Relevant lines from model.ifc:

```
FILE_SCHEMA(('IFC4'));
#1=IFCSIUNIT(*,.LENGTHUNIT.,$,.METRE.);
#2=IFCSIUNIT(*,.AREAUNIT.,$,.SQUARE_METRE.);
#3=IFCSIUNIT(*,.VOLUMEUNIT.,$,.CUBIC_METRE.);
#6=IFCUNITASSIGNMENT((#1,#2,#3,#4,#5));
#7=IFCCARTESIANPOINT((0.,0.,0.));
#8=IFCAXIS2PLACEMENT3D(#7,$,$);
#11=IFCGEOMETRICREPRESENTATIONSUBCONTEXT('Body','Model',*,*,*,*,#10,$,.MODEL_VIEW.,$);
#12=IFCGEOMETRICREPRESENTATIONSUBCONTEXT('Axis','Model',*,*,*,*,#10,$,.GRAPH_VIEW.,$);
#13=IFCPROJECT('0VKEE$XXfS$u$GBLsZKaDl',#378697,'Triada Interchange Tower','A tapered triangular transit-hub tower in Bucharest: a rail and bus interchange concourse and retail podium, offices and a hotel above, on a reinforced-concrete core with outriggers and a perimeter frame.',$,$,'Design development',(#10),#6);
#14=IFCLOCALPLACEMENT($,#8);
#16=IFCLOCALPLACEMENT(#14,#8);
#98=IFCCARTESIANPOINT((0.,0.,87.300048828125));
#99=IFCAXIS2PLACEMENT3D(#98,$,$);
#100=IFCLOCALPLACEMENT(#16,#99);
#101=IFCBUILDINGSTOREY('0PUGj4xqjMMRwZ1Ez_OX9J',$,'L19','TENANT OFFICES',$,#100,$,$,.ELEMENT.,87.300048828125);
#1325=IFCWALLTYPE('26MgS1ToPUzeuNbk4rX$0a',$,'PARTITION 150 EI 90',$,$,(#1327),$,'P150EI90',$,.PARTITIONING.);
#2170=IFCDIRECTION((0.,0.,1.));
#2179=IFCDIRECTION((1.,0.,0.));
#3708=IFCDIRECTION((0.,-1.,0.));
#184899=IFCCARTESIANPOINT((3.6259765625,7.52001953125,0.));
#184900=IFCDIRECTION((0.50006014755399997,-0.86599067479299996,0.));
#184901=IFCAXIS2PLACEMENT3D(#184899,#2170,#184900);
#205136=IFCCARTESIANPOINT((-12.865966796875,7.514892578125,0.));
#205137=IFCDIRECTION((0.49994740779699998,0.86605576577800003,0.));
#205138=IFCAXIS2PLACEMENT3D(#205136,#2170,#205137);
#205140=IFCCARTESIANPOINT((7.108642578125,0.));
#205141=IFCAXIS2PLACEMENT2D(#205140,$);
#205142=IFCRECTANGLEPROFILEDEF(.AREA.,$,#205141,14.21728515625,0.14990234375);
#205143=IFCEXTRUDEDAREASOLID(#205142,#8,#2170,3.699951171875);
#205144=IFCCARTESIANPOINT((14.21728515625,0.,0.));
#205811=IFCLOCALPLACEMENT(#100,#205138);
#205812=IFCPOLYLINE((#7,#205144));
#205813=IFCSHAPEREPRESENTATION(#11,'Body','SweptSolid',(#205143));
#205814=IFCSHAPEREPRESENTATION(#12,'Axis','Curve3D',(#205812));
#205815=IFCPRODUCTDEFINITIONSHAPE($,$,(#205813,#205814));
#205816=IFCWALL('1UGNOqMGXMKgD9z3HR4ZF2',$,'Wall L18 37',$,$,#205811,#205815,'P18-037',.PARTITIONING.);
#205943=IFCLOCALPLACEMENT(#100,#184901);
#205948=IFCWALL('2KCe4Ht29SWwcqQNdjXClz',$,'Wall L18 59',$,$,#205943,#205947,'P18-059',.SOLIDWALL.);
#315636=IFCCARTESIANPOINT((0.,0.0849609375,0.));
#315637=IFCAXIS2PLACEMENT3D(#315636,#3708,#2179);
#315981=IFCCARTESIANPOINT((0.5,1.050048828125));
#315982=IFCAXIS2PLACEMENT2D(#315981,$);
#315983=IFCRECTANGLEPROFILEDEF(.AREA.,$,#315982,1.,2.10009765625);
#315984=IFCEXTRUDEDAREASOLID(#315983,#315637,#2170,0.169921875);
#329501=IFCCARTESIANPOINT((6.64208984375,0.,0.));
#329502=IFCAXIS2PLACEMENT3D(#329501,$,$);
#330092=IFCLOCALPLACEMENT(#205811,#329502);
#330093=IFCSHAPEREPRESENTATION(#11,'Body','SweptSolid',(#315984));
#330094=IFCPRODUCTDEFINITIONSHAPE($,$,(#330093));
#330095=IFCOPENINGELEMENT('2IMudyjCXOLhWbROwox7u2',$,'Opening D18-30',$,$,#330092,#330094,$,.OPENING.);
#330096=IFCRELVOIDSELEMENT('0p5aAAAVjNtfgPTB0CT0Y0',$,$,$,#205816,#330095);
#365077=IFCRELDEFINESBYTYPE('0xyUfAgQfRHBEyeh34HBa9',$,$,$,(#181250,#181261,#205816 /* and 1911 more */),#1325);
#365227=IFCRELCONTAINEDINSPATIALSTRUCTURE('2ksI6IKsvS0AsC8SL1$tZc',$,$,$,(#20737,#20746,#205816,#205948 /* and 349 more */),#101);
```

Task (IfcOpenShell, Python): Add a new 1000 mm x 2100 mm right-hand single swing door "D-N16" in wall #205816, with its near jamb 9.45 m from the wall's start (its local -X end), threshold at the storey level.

```python
import numpy as np
import ifcopenshell
import ifcopenshell.api.feature
import ifcopenshell.api.geometry
import ifcopenshell.api.root
import ifcopenshell.api.spatial
import ifcopenshell.geom
import ifcopenshell.util.element
import ifcopenshell.util.placement
import ifcopenshell.util.representation
import ifcopenshell.util.shape
import ifcopenshell.util.unit

model = ifcopenshell.open("model.ifc")
unit_scale = ifcopenshell.util.unit.calculate_unit_scale(model)
settings = ifcopenshell.geom.settings()


def volume(element):
    """Net volume in cubic metres, openings subtracted."""
    shape = ifcopenshell.geom.create_shape(settings, element)
    return ifcopenshell.util.shape.get_volume(shape.geometry)


wall = model.by_id(205816)
storey = ifcopenshell.util.element.get_container(wall, ifc_class="IfcBuildingStorey")
context = ifcopenshell.util.representation.get_context(model, "Model", "Body", "MODEL_VIEW")
before = volume(wall)

width, height, from_end, sill = 1, 2.1, 9.45, 0.0  # metres

# The wall runs along its own X axis, and the end named is its -X end.
wall_shape = ifcopenshell.geom.create_shape(settings, wall)
x, y, z = ifcopenshell.util.shape.get_vertices(wall_shape.geometry).T
start = x.min() + from_end
face, thickness = float(y.min()), float(y.max() - y.min())
wall_matrix = ifcopenshell.util.placement.get_local_placement(wall.ObjectPlacement)
level = ifcopenshell.util.placement.get_local_placement(storey.ObjectPlacement)[2, 3]


def in_wall(x, y):
    """Placement at x, y metres in the wall's axes, at sill height."""
    matrix = wall_matrix.copy()
    matrix[:, 3] = wall_matrix @ np.array([x / unit_scale, y / unit_scale, 0.0, 1.0])
    matrix[2, 3] = level + sill / unit_scale
    return matrix


# Opening: a box that overshoots both wall faces by 50 mm.
opening = ifcopenshell.api.root.create_entity(model, ifc_class="IfcOpeningElement", predefined_type="OPENING")
box = ifcopenshell.api.geometry.add_wall_representation(
    model, context=context, length=width, height=height, thickness=thickness + 0.1
)
ifcopenshell.api.geometry.assign_representation(model, product=opening, representation=box)
ifcopenshell.api.geometry.edit_object_placement(model, product=opening, matrix=in_wall(start, face - 0.05), is_si=False)
ifcopenshell.api.feature.add_feature(model, feature=opening, element=wall)

door = ifcopenshell.api.root.create_entity(model, ifc_class="IfcDoor", name="D-N16", predefined_type="DOOR")
door.OverallWidth, door.OverallHeight = width / unit_scale, height / unit_scale
door.OperationType = "SINGLE_SWING_RIGHT"
body = ifcopenshell.api.geometry.add_door_representation(
    model,
    context=context,
    overall_width=door.OverallWidth,
    overall_height=door.OverallHeight,
    operation_type="SINGLE_SWING_RIGHT",
    lining_properties={"LiningDepth": thickness / unit_scale, "ThresholdDepth": thickness / unit_scale},
)
ifcopenshell.api.geometry.assign_representation(model, product=door, representation=body)
ifcopenshell.api.spatial.assign_container(model, products=[door], relating_structure=storey)
ifcopenshell.api.feature.add_filling(model, opening=opening, element=door)

# The lining spans the wall, so the door starts at the wall face.
ifcopenshell.api.geometry.edit_object_placement(model, product=door, matrix=in_wall(start, face), is_si=False)

after = volume(wall)

print(f"wall volume {before:.3f} -> {after:.3f} m3")

model.write("model_edited.ifc")
```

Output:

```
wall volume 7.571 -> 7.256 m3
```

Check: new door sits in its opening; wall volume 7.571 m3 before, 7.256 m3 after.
